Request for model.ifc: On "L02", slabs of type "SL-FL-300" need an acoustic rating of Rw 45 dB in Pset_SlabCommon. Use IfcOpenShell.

First a look at what the model holds.

```python
import ifcopenshell
import ifcopenshell.util.element

model = ifcopenshell.open("model.ifc")
print(model.schema)
storey = next(s for s in model.by_type("IfcBuildingStorey") if s.Name == "L02")
slabs = [e for e in ifcopenshell.util.element.get_decomposition(storey) if e.is_a("IfcSlab")]
seen = {}
for e in slabs:
    element_type = ifcopenshell.util.element.get_type(e)
    key = (element_type.Name if element_type != e and element_type else None, ifcopenshell.util.element.get_pset(e, "Pset_SlabCommon", "AcousticRating"))
    seen[key] = seen.get(key, 0) + 1
for (name, value), count in sorted(seen.items(), key=str):
    print(count, "x", name, "|", value)
```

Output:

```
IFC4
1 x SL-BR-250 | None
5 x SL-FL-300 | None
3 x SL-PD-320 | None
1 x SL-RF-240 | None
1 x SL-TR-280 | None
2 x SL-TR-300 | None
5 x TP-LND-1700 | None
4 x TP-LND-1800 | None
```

```python
import ifcopenshell
import ifcopenshell.api.pset
import ifcopenshell.util.element

model = ifcopenshell.open("model.ifc")

storey = next(s for s in model.by_type("IfcBuildingStorey") if s.Name == "L02")
slabs = [e for e in ifcopenshell.util.element.get_decomposition(storey) if e.is_a("IfcSlab")]

count = 0
for e in slabs:
    element_type = ifcopenshell.util.element.get_type(e)
    if element_type in (None, e) or element_type.Name != "SL-FL-300":
        continue
    # add_pset returns the element's existing set when there is one.
    pset = ifcopenshell.api.pset.add_pset(model, product=e, name="Pset_SlabCommon")
    ifcopenshell.api.pset.edit_pset(model, pset=pset, properties={"AcousticRating": "Rw 45 dB"})
    count += 1

print(count, "slabs updated")

model.write("model_updated.ifc")
```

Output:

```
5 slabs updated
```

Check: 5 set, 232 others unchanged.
